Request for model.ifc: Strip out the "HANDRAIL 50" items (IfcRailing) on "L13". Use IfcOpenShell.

First a look at what the model holds.

```python
import ifcopenshell
import ifcopenshell.util.element

model = ifcopenshell.open("model.ifc")
print(model.schema)
storey = next(s for s in model.by_type("IfcBuildingStorey") if s.Name == "L13")
railings = [e for e in ifcopenshell.util.element.get_decomposition(storey) if e.is_a("IfcRailing")]
seen = {}
for e in railings:
    element_type = ifcopenshell.util.element.get_type(e)
    name = element_type.Name if element_type not in (None, e) else None
    seen[name] = seen.get(name, 0) + 1
for name, count in sorted(seen.items(), key=str):
    print(count, "x", name)
```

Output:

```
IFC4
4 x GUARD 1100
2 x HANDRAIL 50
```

```python
import ifcopenshell
import ifcopenshell.api.root
import ifcopenshell.util.element

model = ifcopenshell.open("model.ifc")

storey = next(s for s in model.by_type("IfcBuildingStorey") if s.Name == "L13")
railings = [e for e in ifcopenshell.util.element.get_decomposition(storey) if e.is_a("IfcRailing")]
targets = [e for e in railings if (t := ifcopenshell.util.element.get_type(e)) not in (None, e) and t.Name == "HANDRAIL 50"]

for e in targets:
    ifcopenshell.api.root.remove_product(model, product=e)
print(len(targets), "removed")

model.write("model_edited.ifc")
```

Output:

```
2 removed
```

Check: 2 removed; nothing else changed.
